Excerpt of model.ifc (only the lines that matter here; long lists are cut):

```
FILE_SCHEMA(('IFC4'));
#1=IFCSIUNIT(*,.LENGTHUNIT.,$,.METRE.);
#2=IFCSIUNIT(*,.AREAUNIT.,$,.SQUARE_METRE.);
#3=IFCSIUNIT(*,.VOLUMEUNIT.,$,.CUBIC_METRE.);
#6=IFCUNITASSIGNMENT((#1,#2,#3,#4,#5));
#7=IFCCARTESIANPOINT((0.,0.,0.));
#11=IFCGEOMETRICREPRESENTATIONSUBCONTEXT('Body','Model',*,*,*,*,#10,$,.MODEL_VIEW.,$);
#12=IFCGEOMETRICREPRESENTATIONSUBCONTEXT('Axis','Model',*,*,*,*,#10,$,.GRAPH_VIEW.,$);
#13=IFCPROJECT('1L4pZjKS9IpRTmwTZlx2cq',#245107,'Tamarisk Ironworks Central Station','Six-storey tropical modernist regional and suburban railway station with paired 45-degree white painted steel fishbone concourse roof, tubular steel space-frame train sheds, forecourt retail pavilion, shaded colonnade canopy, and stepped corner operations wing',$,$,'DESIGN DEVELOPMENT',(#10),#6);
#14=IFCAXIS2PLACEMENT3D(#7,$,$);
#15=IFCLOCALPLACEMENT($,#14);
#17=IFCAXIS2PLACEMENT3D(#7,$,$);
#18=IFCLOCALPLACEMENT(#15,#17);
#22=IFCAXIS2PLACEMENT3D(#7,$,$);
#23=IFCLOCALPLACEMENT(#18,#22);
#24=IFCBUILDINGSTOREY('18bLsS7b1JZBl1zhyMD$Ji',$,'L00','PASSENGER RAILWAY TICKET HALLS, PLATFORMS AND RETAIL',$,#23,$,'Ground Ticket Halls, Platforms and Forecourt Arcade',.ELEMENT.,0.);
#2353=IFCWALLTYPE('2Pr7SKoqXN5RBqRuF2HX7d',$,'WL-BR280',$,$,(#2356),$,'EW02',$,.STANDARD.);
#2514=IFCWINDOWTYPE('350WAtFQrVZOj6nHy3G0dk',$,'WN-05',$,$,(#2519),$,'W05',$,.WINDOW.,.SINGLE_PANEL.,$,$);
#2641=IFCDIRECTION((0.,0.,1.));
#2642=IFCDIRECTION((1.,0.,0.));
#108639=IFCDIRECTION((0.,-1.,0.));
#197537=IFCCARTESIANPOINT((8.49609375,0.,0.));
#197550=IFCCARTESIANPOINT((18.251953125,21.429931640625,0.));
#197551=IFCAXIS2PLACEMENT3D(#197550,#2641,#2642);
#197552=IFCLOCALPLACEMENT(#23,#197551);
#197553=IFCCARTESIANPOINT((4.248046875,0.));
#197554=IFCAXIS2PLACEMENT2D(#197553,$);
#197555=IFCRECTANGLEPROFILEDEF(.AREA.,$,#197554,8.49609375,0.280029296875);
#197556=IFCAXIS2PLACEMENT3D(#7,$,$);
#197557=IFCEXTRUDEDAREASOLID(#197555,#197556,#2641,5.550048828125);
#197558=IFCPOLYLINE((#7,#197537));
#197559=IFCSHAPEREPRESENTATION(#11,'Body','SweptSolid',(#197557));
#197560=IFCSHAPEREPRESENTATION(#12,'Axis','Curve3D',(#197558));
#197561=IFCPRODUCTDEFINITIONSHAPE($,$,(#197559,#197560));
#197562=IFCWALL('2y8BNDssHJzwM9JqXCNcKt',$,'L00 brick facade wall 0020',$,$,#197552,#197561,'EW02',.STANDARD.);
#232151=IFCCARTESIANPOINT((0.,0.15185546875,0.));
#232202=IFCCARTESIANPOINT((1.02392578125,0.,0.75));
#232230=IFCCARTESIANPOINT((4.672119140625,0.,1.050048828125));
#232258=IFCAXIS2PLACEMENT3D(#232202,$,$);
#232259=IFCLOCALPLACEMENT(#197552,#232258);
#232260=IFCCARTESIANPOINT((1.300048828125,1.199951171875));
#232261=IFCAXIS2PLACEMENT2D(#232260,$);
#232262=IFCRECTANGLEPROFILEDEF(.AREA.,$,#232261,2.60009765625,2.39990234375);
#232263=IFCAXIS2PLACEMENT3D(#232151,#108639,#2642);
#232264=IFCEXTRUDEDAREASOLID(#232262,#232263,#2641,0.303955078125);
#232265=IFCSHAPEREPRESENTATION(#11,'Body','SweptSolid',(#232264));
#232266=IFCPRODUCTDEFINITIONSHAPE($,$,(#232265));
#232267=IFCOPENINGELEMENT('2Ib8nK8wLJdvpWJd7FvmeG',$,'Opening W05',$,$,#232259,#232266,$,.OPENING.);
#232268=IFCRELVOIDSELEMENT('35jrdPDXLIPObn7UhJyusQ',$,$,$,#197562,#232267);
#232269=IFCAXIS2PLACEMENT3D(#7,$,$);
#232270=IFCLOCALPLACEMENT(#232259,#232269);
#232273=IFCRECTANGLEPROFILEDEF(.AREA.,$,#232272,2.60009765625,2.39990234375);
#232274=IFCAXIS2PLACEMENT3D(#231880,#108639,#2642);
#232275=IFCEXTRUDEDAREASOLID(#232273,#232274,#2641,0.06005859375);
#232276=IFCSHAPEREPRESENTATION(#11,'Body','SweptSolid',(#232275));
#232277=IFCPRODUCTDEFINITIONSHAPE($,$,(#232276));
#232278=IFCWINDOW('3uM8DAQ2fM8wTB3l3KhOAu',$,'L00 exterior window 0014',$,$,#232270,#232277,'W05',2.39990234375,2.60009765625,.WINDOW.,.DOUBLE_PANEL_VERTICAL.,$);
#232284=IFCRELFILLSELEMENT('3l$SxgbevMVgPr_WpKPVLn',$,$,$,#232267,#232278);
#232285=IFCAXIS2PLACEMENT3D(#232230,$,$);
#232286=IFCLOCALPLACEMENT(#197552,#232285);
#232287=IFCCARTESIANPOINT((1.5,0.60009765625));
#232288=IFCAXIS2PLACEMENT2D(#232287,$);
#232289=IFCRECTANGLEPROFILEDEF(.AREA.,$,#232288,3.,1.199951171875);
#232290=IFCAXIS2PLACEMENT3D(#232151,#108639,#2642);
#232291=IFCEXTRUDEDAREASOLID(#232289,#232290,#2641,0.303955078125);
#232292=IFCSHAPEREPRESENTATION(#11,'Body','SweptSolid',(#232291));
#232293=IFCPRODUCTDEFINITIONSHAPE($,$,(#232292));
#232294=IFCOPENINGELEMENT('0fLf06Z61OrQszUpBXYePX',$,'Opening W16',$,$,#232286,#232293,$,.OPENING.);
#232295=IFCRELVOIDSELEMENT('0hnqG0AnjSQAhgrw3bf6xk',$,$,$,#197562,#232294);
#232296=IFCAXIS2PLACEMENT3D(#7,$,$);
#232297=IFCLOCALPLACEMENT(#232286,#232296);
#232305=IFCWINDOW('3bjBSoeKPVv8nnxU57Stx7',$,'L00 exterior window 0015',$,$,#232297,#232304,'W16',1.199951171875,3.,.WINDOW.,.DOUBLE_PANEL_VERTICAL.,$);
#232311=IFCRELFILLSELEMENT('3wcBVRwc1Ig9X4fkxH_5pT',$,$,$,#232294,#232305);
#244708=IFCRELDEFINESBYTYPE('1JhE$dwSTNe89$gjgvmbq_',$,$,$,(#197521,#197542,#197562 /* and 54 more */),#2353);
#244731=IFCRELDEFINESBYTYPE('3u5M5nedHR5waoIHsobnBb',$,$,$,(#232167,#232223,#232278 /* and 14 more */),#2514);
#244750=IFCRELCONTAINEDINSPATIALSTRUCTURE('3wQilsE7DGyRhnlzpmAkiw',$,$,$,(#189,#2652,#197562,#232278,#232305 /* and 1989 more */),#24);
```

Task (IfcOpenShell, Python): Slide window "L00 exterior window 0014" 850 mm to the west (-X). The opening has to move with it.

```python
import ifcopenshell
import ifcopenshell.api.geometry
import ifcopenshell.util.placement
import ifcopenshell.util.unit

model = ifcopenshell.open("model.ifc")
unit_scale = ifcopenshell.util.unit.calculate_unit_scale(model)

window = model.by_guid("3uM8DAQ2fM8wTB3l3KhOAu")
opening = window.FillsVoids[0].RelatingOpeningElement
wall = opening.VoidsElements[0].RelatingBuildingElement

wall_matrix = ifcopenshell.util.placement.get_local_placement(wall.ObjectPlacement)
shift = wall_matrix[:3, 0] * -0.85 / unit_scale
before = ifcopenshell.util.placement.get_local_placement(window.ObjectPlacement)[:3, 3].copy()

# The window is placed relative to its opening, so it follows when the opening moves.
matrix = ifcopenshell.util.placement.get_local_placement(opening.ObjectPlacement)
matrix[:3, 3] += shift
ifcopenshell.api.geometry.edit_object_placement(
    model, product=opening, matrix=matrix, is_si=False, should_transform_children=True
)

after = ifcopenshell.util.placement.get_local_placement(window.ObjectPlacement)[:3, 3]
print("window moved by", (after - before).round(3) + 0.0)

model.write("model_updated.ifc")
```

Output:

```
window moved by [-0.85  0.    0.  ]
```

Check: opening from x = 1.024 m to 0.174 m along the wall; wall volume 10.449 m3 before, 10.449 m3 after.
